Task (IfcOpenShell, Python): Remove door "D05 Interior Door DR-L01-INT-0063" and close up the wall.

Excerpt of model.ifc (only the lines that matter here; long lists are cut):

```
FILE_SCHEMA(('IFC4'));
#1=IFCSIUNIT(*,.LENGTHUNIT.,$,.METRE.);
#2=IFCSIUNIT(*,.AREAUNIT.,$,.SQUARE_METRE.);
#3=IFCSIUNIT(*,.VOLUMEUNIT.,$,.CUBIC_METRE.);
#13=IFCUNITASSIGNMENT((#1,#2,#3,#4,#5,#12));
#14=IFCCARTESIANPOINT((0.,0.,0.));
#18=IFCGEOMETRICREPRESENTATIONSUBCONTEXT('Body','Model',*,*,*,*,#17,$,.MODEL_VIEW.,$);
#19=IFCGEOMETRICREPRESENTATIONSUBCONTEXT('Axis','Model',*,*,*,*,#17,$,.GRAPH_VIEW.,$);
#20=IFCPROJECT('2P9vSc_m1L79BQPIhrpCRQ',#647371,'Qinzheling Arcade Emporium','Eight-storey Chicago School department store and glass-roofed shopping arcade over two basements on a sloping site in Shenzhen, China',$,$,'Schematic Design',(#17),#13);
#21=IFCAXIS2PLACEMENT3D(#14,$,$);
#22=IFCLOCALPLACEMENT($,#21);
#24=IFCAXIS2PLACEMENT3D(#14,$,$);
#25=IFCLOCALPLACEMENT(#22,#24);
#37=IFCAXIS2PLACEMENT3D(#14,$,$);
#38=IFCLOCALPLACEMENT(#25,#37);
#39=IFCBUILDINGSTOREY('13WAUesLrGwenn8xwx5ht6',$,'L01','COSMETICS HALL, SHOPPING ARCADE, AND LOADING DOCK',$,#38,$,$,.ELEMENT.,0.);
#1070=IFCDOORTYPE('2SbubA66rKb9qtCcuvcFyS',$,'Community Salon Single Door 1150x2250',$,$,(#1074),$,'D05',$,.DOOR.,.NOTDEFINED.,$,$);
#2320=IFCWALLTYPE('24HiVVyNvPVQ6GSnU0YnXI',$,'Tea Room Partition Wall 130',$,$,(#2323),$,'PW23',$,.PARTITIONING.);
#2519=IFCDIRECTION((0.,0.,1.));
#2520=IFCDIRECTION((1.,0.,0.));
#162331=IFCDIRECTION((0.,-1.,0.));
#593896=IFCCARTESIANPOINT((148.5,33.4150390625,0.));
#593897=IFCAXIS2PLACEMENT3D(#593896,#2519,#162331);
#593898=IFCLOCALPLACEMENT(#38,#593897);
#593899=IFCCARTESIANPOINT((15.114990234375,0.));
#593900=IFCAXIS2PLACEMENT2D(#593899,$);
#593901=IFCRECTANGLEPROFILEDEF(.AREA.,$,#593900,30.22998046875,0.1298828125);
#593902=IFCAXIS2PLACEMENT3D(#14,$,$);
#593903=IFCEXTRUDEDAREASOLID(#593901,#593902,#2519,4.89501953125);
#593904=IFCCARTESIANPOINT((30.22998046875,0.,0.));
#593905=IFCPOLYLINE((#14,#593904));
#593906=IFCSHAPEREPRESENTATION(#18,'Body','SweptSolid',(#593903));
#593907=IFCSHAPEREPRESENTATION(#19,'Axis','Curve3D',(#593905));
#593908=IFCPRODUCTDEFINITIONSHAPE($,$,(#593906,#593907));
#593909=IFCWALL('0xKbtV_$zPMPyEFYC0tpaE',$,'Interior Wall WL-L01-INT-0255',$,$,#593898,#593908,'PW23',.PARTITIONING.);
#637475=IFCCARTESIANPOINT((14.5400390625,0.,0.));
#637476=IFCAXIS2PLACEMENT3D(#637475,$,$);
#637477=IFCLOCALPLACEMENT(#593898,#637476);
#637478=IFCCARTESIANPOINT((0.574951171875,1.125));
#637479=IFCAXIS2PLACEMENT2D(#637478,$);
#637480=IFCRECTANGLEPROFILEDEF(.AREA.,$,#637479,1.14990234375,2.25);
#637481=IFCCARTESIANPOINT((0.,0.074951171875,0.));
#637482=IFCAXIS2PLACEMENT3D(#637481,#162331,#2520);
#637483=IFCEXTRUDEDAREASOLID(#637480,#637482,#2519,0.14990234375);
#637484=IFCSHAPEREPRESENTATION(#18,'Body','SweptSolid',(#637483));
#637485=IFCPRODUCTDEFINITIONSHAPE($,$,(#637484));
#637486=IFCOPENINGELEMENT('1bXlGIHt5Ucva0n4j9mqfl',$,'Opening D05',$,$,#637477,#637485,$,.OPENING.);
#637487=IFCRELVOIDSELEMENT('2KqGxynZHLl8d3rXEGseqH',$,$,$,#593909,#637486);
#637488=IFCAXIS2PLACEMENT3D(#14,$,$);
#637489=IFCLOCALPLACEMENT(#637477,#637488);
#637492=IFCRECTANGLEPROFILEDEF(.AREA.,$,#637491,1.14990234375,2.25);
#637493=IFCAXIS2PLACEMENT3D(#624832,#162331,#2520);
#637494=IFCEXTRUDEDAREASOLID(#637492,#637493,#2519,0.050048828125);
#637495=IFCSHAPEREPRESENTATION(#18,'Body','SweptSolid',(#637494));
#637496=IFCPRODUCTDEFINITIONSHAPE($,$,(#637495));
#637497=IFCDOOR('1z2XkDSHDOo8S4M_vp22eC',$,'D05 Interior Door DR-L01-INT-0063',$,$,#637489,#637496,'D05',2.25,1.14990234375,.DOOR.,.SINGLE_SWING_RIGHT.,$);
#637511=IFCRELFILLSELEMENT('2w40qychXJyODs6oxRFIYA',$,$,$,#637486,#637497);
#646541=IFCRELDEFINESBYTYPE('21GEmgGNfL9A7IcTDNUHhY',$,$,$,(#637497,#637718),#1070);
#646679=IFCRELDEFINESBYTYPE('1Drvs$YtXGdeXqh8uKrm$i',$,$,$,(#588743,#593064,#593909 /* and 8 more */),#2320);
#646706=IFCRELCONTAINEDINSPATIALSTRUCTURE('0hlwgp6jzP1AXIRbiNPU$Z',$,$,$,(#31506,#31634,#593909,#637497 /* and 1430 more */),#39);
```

```python
import ifcopenshell
import ifcopenshell.api.feature
import ifcopenshell.api.root
import ifcopenshell.geom
import ifcopenshell.util.shape

model = ifcopenshell.open("model.ifc")
settings = ifcopenshell.geom.settings()


def volume(element):
    """Net volume in cubic metres, openings subtracted."""
    shape = ifcopenshell.geom.create_shape(settings, element)
    return ifcopenshell.util.shape.get_volume(shape.geometry)


door = model.by_id(637497)
opening = door.FillsVoids[0].RelatingOpeningElement
wall = opening.VoidsElements[0].RelatingBuildingElement
before = volume(wall)

ifcopenshell.api.root.remove_product(model, product=door)
ifcopenshell.api.feature.remove_feature(model, feature=opening)

after = volume(wall)

print(f"wall volume {before:.3f} -> {after:.3f} m3")

model.write("model_edited.ifc")
```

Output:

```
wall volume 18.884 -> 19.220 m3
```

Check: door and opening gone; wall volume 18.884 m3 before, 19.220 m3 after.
